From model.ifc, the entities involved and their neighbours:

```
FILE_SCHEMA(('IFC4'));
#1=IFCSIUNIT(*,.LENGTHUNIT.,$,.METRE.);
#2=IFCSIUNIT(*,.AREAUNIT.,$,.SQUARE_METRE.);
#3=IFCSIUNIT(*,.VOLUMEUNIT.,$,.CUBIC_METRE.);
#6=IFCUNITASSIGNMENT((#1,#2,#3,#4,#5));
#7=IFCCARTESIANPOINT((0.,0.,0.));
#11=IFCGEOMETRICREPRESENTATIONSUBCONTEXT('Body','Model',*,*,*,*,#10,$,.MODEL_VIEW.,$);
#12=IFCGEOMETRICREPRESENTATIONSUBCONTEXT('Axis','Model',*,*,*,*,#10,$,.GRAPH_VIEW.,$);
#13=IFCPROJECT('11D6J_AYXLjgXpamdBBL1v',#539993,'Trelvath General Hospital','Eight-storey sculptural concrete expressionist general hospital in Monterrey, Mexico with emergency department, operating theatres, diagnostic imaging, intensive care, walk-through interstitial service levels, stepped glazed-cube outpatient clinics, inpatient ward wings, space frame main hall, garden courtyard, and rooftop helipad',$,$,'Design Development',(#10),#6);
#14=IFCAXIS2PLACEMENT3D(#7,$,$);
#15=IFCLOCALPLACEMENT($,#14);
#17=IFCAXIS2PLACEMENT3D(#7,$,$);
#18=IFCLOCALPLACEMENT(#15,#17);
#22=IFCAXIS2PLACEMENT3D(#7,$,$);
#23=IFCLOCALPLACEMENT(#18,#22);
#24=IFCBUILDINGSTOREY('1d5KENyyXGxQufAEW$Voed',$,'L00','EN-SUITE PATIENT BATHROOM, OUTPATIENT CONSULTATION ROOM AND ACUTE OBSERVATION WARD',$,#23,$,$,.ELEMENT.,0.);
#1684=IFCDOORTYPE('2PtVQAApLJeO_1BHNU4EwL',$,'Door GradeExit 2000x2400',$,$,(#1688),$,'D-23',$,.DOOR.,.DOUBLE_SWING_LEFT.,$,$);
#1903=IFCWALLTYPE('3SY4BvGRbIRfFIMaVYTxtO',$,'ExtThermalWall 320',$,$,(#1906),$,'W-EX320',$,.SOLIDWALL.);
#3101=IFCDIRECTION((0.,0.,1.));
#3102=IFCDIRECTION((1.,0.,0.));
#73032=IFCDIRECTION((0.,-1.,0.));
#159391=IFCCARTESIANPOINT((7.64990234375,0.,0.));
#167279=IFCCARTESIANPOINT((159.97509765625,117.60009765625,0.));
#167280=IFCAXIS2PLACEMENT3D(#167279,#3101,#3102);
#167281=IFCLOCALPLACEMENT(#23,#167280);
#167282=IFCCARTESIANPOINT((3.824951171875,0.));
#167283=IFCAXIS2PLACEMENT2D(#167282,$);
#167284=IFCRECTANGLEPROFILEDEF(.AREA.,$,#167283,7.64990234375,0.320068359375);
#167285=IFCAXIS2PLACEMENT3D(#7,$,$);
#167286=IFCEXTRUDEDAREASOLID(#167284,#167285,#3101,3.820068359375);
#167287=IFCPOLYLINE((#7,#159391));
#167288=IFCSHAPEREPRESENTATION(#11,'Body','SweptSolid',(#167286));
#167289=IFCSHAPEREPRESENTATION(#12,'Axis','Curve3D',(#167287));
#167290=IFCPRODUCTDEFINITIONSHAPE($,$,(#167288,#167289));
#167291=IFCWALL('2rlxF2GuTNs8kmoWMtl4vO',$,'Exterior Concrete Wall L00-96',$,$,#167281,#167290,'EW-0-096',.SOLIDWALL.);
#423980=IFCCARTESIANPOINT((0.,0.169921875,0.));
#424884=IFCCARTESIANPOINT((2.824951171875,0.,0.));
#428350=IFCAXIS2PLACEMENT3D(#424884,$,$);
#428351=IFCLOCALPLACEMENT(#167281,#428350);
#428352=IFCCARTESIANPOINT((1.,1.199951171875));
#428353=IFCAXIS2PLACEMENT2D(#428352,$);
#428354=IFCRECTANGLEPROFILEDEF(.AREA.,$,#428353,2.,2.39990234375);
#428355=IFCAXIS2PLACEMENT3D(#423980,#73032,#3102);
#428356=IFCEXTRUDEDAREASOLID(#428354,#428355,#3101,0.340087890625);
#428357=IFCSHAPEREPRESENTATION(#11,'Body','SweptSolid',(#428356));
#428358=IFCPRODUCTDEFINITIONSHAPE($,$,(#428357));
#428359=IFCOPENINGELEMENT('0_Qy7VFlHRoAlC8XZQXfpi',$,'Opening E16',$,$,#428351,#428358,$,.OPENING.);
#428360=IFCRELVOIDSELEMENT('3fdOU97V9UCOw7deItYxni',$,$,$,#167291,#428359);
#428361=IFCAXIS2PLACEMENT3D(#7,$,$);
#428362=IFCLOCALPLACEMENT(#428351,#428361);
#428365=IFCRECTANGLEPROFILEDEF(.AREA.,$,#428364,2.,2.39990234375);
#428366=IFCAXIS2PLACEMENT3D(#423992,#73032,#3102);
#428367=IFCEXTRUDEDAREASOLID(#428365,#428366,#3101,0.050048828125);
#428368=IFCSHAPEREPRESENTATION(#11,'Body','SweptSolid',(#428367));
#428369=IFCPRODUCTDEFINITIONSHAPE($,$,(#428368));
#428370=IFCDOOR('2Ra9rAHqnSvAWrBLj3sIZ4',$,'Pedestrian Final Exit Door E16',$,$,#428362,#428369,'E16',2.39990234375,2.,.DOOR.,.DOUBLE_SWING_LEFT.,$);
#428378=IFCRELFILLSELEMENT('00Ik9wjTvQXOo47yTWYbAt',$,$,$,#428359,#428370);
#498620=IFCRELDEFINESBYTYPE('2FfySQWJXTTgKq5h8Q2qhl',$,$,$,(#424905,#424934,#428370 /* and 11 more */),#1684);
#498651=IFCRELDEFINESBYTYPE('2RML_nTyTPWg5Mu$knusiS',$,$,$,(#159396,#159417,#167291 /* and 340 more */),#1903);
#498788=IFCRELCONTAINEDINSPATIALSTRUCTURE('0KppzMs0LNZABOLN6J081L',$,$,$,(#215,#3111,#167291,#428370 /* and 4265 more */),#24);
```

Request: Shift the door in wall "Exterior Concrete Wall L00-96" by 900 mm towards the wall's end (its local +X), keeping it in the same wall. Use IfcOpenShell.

```python
import ifcopenshell
import ifcopenshell.api.geometry
import ifcopenshell.util.placement
import ifcopenshell.util.unit

model = ifcopenshell.open("model.ifc")
unit_scale = ifcopenshell.util.unit.calculate_unit_scale(model)

door = model.by_id(428370)
opening = door.FillsVoids[0].RelatingOpeningElement
wall = opening.VoidsElements[0].RelatingBuildingElement

wall_matrix = ifcopenshell.util.placement.get_local_placement(wall.ObjectPlacement)
shift = wall_matrix[:3, 0] * 0.9 / unit_scale
before = ifcopenshell.util.placement.get_local_placement(door.ObjectPlacement)[:3, 3].copy()

# The door is placed relative to its opening, so it follows when the opening moves.
matrix = ifcopenshell.util.placement.get_local_placement(opening.ObjectPlacement)
matrix[:3, 3] += shift
ifcopenshell.api.geometry.edit_object_placement(
    model, product=opening, matrix=matrix, is_si=False, should_transform_children=True
)

after = ifcopenshell.util.placement.get_local_placement(door.ObjectPlacement)[:3, 3]
print("door moved by", (after - before).round(3) + 0.0)

model.write("model_updated.ifc")
```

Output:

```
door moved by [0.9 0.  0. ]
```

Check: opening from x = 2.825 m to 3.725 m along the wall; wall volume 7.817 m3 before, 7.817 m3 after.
